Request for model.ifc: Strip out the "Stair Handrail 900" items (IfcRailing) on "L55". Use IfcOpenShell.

First a look at what the model holds.

```python
import ifcopenshell
import ifcopenshell.util.element

model = ifcopenshell.open("model.ifc")
print(model.schema)
storey = next(s for s in model.by_type("IfcBuildingStorey") if s.Name == "L55")
railings = [e for e in ifcopenshell.util.element.get_decomposition(storey) if e.is_a("IfcRailing")]
seen = {}
for e in railings:
    element_type = ifcopenshell.util.element.get_type(e)
    name = element_type.Name if element_type not in (None, e) else None
    seen[name] = seen.get(name, 0) + 1
for name, count in sorted(seen.items(), key=str):
    print(count, "x", name)
```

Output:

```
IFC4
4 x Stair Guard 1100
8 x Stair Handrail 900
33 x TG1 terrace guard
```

```python
import ifcopenshell
import ifcopenshell.api.root
import ifcopenshell.util.element

model = ifcopenshell.open("model.ifc")

storey = next(s for s in model.by_type("IfcBuildingStorey") if s.Name == "L55")
railings = [e for e in ifcopenshell.util.element.get_decomposition(storey) if e.is_a("IfcRailing")]
targets = [e for e in railings if (t := ifcopenshell.util.element.get_type(e)) not in (None, e) and t.Name == "Stair Handrail 900"]

for e in targets:
    ifcopenshell.api.root.remove_product(model, product=e)
print(len(targets), "removed")

model.write("model-out.ifc")
```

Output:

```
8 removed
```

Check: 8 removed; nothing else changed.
